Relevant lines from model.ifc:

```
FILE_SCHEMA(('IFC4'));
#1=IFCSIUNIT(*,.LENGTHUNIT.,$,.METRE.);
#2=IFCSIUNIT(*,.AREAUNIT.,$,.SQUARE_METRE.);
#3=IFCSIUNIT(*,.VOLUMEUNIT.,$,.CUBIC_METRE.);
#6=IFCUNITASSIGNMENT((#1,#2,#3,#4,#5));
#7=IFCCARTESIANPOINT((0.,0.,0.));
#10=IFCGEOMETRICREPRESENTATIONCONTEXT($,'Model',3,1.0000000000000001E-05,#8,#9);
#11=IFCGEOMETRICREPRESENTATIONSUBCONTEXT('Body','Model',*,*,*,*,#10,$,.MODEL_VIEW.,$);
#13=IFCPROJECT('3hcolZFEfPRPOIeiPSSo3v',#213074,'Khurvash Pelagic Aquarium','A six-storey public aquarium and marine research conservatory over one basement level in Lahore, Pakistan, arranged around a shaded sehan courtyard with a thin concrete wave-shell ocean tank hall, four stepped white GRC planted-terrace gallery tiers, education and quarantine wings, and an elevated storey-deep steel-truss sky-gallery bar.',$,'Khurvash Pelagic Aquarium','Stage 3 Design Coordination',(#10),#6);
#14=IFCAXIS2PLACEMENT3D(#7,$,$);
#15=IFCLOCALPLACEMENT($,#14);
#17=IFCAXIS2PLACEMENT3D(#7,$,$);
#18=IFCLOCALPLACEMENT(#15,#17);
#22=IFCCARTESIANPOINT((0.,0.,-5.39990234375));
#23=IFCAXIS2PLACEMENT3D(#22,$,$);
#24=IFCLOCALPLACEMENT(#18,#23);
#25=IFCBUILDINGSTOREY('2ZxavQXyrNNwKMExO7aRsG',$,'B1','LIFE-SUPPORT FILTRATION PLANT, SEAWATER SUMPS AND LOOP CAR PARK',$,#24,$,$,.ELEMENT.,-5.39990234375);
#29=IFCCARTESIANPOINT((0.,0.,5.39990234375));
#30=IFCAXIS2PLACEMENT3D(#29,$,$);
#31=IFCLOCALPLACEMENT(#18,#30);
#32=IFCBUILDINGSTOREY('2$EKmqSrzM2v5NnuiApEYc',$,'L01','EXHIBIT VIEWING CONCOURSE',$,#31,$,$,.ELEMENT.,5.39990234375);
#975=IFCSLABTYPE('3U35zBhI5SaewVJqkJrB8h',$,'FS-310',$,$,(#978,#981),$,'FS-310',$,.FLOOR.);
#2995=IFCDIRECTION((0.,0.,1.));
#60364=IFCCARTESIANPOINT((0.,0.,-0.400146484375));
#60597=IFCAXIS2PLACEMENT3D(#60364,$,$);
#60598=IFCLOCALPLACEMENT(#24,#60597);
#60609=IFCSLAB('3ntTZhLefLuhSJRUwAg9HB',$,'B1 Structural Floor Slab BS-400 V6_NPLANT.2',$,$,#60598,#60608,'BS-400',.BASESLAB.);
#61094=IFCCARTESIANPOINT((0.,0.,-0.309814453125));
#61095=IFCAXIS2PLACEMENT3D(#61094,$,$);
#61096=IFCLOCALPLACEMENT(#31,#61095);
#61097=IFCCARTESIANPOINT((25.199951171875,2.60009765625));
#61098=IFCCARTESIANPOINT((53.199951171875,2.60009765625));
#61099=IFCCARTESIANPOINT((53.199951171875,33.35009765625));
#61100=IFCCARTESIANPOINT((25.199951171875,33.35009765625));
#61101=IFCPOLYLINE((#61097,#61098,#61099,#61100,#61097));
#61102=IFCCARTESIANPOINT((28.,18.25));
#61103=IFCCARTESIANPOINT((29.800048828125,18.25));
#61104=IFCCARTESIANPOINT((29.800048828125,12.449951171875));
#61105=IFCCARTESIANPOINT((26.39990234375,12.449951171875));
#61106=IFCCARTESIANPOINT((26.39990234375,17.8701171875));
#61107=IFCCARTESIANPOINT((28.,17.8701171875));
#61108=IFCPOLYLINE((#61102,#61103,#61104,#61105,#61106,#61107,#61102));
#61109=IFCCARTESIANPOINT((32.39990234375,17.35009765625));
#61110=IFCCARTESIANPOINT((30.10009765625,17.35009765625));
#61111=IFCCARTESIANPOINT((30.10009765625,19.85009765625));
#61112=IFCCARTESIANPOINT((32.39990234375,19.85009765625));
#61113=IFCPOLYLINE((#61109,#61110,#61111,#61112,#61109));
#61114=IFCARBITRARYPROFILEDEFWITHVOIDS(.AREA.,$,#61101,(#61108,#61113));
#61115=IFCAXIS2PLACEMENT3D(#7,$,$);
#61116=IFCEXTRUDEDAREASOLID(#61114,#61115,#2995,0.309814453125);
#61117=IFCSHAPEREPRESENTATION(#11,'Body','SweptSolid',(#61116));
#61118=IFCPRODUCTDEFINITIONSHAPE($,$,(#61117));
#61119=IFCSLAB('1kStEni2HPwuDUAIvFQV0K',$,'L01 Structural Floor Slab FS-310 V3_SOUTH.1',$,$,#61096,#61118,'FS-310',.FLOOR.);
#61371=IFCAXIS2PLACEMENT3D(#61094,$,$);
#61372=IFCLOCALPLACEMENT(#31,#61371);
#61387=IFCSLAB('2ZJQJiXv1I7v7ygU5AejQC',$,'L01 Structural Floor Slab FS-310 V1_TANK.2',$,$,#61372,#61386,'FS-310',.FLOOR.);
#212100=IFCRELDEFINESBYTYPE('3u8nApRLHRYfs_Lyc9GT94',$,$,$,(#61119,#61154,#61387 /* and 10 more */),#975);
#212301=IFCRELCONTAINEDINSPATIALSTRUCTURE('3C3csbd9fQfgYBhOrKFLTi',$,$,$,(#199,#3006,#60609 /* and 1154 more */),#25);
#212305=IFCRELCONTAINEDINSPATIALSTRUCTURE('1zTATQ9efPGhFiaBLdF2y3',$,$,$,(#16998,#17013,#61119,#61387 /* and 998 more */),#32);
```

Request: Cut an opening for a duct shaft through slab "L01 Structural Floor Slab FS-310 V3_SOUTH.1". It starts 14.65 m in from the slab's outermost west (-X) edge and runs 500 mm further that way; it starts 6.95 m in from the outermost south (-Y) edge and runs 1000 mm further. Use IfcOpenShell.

```python
import numpy as np
import ifcopenshell
import ifcopenshell.api.feature
import ifcopenshell.api.geometry
import ifcopenshell.api.root
import ifcopenshell.geom
import ifcopenshell.util.placement
import ifcopenshell.util.representation
import ifcopenshell.util.shape
import ifcopenshell.util.unit

model = ifcopenshell.open("model.ifc")
unit_scale = ifcopenshell.util.unit.calculate_unit_scale(model)
settings = ifcopenshell.geom.settings()


def volume(element):
    """Net volume in cubic metres, openings subtracted."""
    shape = ifcopenshell.geom.create_shape(settings, element)
    return ifcopenshell.util.shape.get_volume(shape.geometry)


slab = model.by_guid("1kStEni2HPwuDUAIvFQV0K")
before = volume(slab)

# Extent in the slab's own axes, in metres. The edges named are its -X and -Y sides.
slab_shape = ifcopenshell.geom.create_shape(settings, slab)
vertices = ifcopenshell.util.shape.get_vertices(slab_shape.geometry)
x_min, y_min, bottom = vertices.min(axis=0)
top = vertices[:, 2].max()

opening = ifcopenshell.api.root.create_entity(model, ifc_class="IfcOpeningElement", name="Duct shaft opening", predefined_type="OPENING")
context = ifcopenshell.util.representation.get_context(model, "Model", "Body", "MODEL_VIEW")
width, depth = 0.5, 1
outline = [(0.0, 0.0), (width, 0.0), (width, depth), (0.0, depth), (0.0, 0.0)]
# Overshoot both faces by 50 mm so the cut is clean.
shape = ifcopenshell.api.geometry.add_slab_representation(
    model, context=context, depth=top - bottom + 0.1, polyline=outline
)
ifcopenshell.api.geometry.assign_representation(model, product=opening, representation=shape)

matrix = ifcopenshell.util.placement.get_local_placement(slab.ObjectPlacement)
matrix[:, 3] = matrix @ np.append(np.array([x_min + 14.65, y_min + 6.95, bottom - 0.05]) / unit_scale, 1.0)
ifcopenshell.api.geometry.edit_object_placement(model, product=opening, matrix=matrix, is_si=False)
ifcopenshell.api.feature.add_feature(model, feature=opening, element=slab)

after = volume(slab)

print(f"slab volume {before:.3f} -> {after:.3f} m3")

model.write("model_v2.ifc")
```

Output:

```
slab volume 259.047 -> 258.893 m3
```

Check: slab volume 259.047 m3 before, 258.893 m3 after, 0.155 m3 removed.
